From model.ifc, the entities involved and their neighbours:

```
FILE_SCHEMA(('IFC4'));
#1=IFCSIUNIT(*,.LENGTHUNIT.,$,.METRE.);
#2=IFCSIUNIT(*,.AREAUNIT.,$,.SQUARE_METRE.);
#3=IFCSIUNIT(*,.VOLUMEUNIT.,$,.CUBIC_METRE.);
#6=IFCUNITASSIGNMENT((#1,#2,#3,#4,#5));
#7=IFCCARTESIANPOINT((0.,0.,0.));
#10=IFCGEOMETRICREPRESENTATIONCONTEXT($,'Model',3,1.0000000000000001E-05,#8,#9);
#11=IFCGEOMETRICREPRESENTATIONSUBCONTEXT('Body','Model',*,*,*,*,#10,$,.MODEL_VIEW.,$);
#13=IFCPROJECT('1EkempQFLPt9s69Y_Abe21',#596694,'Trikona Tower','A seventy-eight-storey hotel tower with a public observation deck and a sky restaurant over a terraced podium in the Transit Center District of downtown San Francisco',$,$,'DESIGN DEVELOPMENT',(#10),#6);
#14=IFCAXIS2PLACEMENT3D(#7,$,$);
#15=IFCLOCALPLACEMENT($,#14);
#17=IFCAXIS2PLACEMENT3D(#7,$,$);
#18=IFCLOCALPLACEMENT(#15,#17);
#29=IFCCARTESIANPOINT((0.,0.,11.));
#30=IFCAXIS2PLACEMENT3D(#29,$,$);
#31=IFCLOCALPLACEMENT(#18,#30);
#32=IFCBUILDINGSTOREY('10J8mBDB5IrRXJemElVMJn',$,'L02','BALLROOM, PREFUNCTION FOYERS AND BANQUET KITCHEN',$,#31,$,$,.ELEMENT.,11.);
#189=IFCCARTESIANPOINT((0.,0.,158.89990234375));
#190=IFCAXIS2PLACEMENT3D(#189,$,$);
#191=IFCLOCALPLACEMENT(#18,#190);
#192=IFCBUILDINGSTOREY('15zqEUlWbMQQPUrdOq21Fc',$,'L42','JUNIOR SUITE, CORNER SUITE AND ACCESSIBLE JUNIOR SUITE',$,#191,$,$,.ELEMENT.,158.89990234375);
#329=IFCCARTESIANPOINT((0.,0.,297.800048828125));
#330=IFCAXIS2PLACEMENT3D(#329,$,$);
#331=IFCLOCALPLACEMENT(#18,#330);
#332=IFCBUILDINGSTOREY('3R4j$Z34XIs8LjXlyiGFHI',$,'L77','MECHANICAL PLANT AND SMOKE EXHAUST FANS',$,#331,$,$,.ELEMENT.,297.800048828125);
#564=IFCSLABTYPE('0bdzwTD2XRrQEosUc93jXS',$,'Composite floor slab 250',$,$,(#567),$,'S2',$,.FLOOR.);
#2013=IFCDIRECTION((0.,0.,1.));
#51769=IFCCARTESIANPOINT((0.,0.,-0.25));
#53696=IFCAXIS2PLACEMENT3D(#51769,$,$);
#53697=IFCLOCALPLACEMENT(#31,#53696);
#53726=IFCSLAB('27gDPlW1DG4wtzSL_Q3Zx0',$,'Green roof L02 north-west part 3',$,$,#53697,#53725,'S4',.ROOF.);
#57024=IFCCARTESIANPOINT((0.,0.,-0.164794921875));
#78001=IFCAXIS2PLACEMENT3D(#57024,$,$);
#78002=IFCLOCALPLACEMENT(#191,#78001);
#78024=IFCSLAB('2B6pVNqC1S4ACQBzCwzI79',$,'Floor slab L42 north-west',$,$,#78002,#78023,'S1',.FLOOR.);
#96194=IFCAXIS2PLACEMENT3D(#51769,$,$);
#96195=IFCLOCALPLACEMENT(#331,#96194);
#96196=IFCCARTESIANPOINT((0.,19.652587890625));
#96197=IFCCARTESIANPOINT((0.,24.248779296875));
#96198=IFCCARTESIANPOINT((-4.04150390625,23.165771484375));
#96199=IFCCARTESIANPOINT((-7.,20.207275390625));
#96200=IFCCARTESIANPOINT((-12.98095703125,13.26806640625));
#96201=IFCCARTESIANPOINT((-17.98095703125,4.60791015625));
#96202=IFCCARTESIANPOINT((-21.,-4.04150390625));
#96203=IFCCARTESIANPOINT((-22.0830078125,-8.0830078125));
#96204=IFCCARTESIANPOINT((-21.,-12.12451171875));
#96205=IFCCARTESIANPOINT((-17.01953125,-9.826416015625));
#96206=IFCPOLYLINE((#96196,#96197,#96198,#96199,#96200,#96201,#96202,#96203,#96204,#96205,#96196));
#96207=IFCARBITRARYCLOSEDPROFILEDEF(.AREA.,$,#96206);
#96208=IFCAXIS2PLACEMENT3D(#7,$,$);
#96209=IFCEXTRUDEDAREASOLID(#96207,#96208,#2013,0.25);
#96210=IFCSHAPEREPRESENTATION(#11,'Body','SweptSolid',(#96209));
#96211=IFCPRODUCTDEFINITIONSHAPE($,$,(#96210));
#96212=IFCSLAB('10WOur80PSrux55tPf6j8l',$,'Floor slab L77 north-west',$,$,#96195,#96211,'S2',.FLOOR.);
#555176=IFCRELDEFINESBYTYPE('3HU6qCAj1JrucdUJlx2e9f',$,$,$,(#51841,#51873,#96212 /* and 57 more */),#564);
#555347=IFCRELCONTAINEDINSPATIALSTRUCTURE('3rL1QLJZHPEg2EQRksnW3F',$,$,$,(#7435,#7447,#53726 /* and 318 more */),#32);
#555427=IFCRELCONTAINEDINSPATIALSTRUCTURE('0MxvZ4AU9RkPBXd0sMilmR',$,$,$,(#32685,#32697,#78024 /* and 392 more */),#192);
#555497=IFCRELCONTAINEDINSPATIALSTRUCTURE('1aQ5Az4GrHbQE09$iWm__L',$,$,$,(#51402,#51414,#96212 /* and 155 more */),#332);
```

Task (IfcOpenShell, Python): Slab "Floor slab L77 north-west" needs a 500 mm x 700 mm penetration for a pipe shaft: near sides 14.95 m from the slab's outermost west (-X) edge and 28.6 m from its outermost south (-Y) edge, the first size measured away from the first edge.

```python
import numpy as np
import ifcopenshell
import ifcopenshell.api.feature
import ifcopenshell.api.geometry
import ifcopenshell.api.root
import ifcopenshell.geom
import ifcopenshell.util.placement
import ifcopenshell.util.representation
import ifcopenshell.util.shape
import ifcopenshell.util.unit

model = ifcopenshell.open("model.ifc")
unit_scale = ifcopenshell.util.unit.calculate_unit_scale(model)
settings = ifcopenshell.geom.settings()


def volume(element):
    """Net volume in cubic metres, openings subtracted."""
    shape = ifcopenshell.geom.create_shape(settings, element)
    return ifcopenshell.util.shape.get_volume(shape.geometry)


slab = model.by_id(96212)
before = volume(slab)

# Extent in the slab's own axes, in metres. The edges named are its -X and -Y sides.
slab_shape = ifcopenshell.geom.create_shape(settings, slab)
vertices = ifcopenshell.util.shape.get_vertices(slab_shape.geometry)
x_min, y_min, bottom = vertices.min(axis=0)
top = vertices[:, 2].max()

opening = ifcopenshell.api.root.create_entity(model, ifc_class="IfcOpeningElement", name="Pipe shaft opening", predefined_type="OPENING")
context = ifcopenshell.util.representation.get_context(model, "Model", "Body", "MODEL_VIEW")
width, depth = 0.5, 0.7
outline = [(0.0, 0.0), (width, 0.0), (width, depth), (0.0, depth), (0.0, 0.0)]
# Overshoot both faces by 50 mm so the cut is clean.
shape = ifcopenshell.api.geometry.add_slab_representation(
    model, context=context, depth=top - bottom + 0.1, polyline=outline
)
ifcopenshell.api.geometry.assign_representation(model, product=opening, representation=shape)

matrix = ifcopenshell.util.placement.get_local_placement(slab.ObjectPlacement)
matrix[:, 3] = matrix @ np.append(np.array([x_min + 14.95, y_min + 28.6, bottom - 0.05]) / unit_scale, 1.0)
ifcopenshell.api.geometry.edit_object_placement(model, product=opening, matrix=matrix, is_si=False)
ifcopenshell.api.feature.add_feature(model, feature=opening, element=slab)

after = volume(slab)

print(f"slab volume {before:.3f} -> {after:.3f} m3")

model.write("model_edited.ifc")
```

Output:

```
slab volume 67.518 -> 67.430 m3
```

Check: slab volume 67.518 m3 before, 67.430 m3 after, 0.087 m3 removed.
